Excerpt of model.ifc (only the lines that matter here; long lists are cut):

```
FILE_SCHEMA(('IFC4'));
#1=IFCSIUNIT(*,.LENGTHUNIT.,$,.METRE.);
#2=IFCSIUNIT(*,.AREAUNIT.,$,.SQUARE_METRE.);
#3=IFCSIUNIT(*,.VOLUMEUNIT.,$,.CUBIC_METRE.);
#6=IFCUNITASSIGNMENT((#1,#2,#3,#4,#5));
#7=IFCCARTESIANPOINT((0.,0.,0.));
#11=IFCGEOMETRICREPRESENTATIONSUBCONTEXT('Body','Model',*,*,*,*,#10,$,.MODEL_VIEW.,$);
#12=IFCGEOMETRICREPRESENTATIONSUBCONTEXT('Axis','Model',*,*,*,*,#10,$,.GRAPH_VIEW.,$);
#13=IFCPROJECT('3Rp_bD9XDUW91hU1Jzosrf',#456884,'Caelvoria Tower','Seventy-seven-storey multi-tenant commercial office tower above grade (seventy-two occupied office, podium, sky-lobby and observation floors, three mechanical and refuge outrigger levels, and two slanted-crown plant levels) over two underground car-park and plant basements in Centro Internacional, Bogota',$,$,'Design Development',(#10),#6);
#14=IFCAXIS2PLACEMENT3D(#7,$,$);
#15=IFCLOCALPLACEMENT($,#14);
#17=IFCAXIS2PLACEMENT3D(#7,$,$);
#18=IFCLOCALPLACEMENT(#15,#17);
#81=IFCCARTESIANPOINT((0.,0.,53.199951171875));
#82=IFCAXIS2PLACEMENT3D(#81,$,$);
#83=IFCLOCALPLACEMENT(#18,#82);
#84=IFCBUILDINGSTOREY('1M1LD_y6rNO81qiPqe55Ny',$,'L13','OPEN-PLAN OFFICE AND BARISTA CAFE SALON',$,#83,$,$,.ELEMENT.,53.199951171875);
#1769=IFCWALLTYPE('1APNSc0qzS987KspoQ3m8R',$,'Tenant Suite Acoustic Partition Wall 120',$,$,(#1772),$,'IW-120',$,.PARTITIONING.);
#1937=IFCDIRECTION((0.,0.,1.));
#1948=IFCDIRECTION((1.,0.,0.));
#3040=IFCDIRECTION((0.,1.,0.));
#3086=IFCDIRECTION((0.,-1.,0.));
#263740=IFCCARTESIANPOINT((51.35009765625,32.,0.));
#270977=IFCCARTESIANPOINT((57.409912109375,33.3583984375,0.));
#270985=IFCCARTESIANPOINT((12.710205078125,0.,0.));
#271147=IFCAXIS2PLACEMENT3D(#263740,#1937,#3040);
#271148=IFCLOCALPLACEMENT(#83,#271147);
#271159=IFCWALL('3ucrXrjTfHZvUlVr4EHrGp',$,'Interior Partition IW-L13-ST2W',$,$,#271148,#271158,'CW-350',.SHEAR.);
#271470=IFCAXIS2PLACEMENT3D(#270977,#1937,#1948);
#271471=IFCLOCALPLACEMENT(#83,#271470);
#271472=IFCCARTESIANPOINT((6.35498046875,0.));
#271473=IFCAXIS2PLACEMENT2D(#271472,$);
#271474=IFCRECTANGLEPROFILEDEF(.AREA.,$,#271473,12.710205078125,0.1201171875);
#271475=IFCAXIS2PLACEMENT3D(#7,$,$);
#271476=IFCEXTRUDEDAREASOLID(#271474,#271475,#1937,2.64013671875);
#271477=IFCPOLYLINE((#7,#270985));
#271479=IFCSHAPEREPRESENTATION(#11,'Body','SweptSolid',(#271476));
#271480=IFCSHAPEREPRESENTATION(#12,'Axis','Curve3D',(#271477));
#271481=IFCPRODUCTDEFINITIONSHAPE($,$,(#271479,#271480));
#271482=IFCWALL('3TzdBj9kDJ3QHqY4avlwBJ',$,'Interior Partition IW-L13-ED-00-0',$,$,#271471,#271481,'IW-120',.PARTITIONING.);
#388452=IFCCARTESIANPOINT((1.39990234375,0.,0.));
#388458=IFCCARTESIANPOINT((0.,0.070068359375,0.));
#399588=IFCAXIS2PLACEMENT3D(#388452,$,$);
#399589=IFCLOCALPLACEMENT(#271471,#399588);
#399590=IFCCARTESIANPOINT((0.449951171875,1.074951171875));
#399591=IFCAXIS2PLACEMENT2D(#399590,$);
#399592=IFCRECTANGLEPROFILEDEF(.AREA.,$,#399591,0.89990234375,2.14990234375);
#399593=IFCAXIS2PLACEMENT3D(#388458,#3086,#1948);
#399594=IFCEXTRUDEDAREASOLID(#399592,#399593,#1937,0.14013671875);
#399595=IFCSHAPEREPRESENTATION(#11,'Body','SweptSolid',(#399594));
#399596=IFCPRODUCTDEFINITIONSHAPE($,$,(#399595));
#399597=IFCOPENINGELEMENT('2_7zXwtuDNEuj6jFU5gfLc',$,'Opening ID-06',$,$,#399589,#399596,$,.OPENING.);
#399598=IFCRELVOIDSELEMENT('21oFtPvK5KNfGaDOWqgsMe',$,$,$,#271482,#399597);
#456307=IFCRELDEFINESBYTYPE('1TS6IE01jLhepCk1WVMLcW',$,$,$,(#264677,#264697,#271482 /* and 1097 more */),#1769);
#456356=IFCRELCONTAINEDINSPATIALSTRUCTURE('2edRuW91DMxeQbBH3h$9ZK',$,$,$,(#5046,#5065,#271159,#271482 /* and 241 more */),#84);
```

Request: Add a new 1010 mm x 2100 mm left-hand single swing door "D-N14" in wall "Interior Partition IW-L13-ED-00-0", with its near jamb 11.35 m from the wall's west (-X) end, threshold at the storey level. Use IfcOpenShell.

```python
import numpy as np
import ifcopenshell
import ifcopenshell.api.feature
import ifcopenshell.api.geometry
import ifcopenshell.api.root
import ifcopenshell.api.spatial
import ifcopenshell.geom
import ifcopenshell.util.element
import ifcopenshell.util.placement
import ifcopenshell.util.representation
import ifcopenshell.util.shape
import ifcopenshell.util.unit

model = ifcopenshell.open("model.ifc")
unit_scale = ifcopenshell.util.unit.calculate_unit_scale(model)
settings = ifcopenshell.geom.settings()


def volume(element):
    """Net volume in cubic metres, openings subtracted."""
    shape = ifcopenshell.geom.create_shape(settings, element)
    return ifcopenshell.util.shape.get_volume(shape.geometry)


wall = model.by_guid("3TzdBj9kDJ3QHqY4avlwBJ")
storey = ifcopenshell.util.element.get_container(wall, ifc_class="IfcBuildingStorey")
context = ifcopenshell.util.representation.get_context(model, "Model", "Body", "MODEL_VIEW")
before = volume(wall)

width, height, from_end, sill = 1.01, 2.1, 11.35, 0.0  # metres

# The wall runs along its own X axis, and the end named is its -X end.
wall_shape = ifcopenshell.geom.create_shape(settings, wall)
x, y, z = ifcopenshell.util.shape.get_vertices(wall_shape.geometry).T
start = x.min() + from_end
face, thickness = float(y.min()), float(y.max() - y.min())
wall_matrix = ifcopenshell.util.placement.get_local_placement(wall.ObjectPlacement)
level = ifcopenshell.util.placement.get_local_placement(storey.ObjectPlacement)[2, 3]


def in_wall(x, y):
    """Placement at x, y metres in the wall's axes, at sill height."""
    matrix = wall_matrix.copy()
    matrix[:, 3] = wall_matrix @ np.array([x / unit_scale, y / unit_scale, 0.0, 1.0])
    matrix[2, 3] = level + sill / unit_scale
    return matrix


# Opening: a box that overshoots both wall faces by 50 mm.
opening = ifcopenshell.api.root.create_entity(model, ifc_class="IfcOpeningElement", predefined_type="OPENING")
box = ifcopenshell.api.geometry.add_wall_representation(
    model, context=context, length=width, height=height, thickness=thickness + 0.1
)
ifcopenshell.api.geometry.assign_representation(model, product=opening, representation=box)
ifcopenshell.api.geometry.edit_object_placement(model, product=opening, matrix=in_wall(start, face - 0.05), is_si=False)
ifcopenshell.api.feature.add_feature(model, feature=opening, element=wall)

door = ifcopenshell.api.root.create_entity(model, ifc_class="IfcDoor", name="D-N14", predefined_type="DOOR")
door.OverallWidth, door.OverallHeight = width / unit_scale, height / unit_scale
door.OperationType = "SINGLE_SWING_LEFT"
body = ifcopenshell.api.geometry.add_door_representation(
    model,
    context=context,
    overall_width=door.OverallWidth,
    overall_height=door.OverallHeight,
    operation_type="SINGLE_SWING_LEFT",
    lining_properties={"LiningDepth": thickness / unit_scale, "ThresholdDepth": thickness / unit_scale},
)
ifcopenshell.api.geometry.assign_representation(model, product=door, representation=body)
ifcopenshell.api.spatial.assign_container(model, products=[door], relating_structure=storey)
ifcopenshell.api.feature.add_filling(model, opening=opening, element=door)

# The lining spans the wall, so the door starts at the wall face.
ifcopenshell.api.geometry.edit_object_placement(model, product=door, matrix=in_wall(start, face), is_si=False)

after = volume(wall)

print(f"wall volume {before:.3f} -> {after:.3f} m3")

model.write("model_updated.ifc")
```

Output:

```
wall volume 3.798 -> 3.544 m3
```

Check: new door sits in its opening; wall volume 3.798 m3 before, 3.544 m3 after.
